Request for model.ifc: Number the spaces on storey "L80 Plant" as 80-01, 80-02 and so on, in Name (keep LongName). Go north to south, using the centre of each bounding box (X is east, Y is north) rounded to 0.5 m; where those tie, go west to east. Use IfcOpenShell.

First a look at what the model holds.

```python
import ifcopenshell
import ifcopenshell.util.element
import ifcopenshell.util.placement

model = ifcopenshell.open("model.ifc")
print(model.schema)
storey = next(s for s in model.by_type("IfcBuildingStorey") if s.Name == "L80 Plant")
spaces = [e for e in ifcopenshell.util.element.get_decomposition(storey) if e.is_a("IfcSpace")]
for e in sorted(spaces, key=lambda e: e.id()):
    origin = ifcopenshell.util.placement.get_local_placement(e.ObjectPlacement)[:3, 3]
    print(e.id(), e.Name, e.LongName, origin.round(2) + 0.0, sep=" | ")
```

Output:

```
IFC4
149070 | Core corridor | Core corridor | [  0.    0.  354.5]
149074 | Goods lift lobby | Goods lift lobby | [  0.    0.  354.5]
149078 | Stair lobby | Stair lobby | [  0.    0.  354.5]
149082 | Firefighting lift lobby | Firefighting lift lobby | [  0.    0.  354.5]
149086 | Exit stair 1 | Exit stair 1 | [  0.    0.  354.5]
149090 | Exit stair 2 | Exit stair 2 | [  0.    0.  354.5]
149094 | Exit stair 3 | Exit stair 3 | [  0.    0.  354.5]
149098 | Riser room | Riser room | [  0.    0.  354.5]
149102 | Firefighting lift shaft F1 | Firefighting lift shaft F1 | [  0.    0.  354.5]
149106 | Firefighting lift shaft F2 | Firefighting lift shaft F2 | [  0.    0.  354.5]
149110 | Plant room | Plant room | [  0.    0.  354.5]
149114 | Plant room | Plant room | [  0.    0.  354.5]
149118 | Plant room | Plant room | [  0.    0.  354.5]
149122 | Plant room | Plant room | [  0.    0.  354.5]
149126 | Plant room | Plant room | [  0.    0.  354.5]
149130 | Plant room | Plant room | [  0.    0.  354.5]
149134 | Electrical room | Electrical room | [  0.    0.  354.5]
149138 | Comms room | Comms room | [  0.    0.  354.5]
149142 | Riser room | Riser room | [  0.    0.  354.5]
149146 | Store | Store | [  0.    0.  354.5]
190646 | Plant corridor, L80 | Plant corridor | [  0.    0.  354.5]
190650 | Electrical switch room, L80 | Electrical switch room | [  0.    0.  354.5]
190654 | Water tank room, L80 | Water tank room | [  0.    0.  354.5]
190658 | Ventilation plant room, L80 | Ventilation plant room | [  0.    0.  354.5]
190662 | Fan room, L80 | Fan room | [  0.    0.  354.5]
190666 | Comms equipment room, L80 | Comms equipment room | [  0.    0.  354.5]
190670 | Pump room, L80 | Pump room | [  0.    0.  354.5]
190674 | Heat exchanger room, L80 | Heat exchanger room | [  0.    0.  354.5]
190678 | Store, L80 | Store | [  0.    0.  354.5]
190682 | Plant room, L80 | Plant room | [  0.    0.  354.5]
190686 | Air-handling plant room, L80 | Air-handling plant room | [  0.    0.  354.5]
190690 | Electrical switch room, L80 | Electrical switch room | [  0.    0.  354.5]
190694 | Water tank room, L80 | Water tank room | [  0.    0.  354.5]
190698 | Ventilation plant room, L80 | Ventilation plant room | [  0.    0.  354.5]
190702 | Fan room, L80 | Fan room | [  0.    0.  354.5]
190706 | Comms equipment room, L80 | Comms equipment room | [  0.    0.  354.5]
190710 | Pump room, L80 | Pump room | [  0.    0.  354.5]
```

```python
import ifcopenshell
import ifcopenshell.geom
import ifcopenshell.util.element
import ifcopenshell.util.shape

model = ifcopenshell.open("model.ifc")
settings = ifcopenshell.geom.settings()
settings.set("use-world-coords", True)


def centre(element):
    shape = ifcopenshell.geom.create_shape(settings, element)
    return ifcopenshell.util.shape.get_bbox_centroid(shape.geometry)


storey = next(s for s in model.by_type("IfcBuildingStorey") if s.Name == "L80 Plant")
spaces = [e for e in ifcopenshell.util.element.get_decomposition(storey) if e.is_a("IfcSpace")]

# Insertion points can sit at a corner or the storey origin, so sort by the geometry (in metres).
centres = {e: centre(e) for e in spaces}
spaces.sort(key=lambda e: (-round(centres[e][1] / 0.5), centres[e][0]))

for i, e in enumerate(spaces, start=1):
    number = f"80-{i:02d}"
    e.Name = number
    print(e.id(), number)

model.write("model_v2.ifc")
```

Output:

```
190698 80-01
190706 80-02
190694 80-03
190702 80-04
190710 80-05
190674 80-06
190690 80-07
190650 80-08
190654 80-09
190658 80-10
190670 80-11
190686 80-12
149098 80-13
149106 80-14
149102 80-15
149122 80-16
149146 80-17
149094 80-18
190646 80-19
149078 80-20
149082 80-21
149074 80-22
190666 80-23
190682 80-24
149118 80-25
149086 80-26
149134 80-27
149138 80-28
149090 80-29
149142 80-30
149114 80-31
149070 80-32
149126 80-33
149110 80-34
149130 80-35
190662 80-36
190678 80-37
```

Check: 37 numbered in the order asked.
